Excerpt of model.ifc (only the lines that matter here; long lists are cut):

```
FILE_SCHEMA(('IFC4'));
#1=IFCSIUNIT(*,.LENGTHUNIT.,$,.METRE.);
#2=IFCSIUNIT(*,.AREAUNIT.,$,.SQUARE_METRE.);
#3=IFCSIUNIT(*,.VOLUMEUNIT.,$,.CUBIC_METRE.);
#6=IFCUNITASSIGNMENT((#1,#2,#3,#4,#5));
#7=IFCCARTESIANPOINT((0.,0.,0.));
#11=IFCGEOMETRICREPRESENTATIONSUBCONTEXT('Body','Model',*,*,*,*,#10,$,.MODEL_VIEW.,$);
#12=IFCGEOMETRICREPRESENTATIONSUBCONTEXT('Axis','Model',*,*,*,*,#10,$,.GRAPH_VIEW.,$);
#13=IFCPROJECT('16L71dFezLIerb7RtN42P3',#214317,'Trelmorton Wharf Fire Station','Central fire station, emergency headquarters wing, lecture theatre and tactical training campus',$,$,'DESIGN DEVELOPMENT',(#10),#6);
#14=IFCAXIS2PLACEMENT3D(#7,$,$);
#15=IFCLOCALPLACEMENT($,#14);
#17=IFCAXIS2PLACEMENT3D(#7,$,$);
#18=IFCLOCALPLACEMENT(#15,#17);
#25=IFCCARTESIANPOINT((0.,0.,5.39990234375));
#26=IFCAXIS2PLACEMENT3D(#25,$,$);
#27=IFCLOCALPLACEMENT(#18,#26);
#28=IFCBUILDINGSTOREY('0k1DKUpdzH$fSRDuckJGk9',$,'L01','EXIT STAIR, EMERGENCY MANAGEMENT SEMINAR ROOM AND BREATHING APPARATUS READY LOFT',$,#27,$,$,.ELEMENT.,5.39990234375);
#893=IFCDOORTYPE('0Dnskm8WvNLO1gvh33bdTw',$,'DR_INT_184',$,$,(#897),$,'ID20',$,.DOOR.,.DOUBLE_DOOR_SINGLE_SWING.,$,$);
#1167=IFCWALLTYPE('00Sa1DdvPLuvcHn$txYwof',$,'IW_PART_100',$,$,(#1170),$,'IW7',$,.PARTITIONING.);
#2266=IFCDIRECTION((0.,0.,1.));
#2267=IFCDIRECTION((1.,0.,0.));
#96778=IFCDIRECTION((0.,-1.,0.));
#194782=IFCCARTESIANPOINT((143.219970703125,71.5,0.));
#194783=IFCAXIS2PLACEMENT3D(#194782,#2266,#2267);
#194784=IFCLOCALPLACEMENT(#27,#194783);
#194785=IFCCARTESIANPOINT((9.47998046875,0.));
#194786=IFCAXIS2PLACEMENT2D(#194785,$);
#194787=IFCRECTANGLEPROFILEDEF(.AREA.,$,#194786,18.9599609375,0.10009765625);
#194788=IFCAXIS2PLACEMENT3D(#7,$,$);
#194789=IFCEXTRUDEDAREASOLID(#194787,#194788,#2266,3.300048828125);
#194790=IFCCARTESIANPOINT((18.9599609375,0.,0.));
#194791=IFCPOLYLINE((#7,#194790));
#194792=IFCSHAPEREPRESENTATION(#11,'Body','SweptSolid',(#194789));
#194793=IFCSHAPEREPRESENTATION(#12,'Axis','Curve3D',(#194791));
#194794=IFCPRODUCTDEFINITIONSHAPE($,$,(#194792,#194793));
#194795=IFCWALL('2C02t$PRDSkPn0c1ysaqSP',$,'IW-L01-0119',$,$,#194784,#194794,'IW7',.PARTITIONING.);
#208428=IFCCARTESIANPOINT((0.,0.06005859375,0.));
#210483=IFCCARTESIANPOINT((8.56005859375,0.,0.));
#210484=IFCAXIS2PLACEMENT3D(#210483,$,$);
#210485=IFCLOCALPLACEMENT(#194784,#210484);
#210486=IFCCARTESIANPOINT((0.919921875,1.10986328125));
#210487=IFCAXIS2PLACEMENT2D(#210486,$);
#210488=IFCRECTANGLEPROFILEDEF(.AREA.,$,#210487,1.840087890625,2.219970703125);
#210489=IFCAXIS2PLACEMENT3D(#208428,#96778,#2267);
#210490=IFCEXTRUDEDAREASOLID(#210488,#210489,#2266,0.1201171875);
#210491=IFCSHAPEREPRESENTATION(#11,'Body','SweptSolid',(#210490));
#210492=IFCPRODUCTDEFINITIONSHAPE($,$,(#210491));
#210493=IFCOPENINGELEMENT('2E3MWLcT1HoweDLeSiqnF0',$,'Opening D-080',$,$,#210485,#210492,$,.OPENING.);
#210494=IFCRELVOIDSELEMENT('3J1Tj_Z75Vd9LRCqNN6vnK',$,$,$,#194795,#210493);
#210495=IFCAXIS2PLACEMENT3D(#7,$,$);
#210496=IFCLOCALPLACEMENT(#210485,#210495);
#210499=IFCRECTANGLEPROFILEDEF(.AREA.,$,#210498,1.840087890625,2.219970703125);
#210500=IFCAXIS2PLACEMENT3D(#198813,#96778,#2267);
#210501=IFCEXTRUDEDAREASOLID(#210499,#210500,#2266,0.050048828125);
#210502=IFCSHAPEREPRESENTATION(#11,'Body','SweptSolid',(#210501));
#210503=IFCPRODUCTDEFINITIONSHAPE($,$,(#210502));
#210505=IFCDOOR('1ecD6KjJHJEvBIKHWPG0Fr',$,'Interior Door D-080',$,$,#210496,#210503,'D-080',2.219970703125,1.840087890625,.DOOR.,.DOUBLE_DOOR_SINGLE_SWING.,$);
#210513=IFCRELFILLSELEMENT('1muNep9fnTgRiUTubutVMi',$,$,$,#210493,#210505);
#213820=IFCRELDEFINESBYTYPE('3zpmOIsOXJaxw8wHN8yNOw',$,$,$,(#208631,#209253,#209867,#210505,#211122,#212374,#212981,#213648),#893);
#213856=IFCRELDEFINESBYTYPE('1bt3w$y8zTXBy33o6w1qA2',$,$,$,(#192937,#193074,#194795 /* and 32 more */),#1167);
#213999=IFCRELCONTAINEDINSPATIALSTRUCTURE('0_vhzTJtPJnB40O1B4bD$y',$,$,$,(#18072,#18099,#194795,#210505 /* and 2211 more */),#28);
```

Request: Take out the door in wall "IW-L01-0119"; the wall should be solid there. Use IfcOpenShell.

```python
import ifcopenshell
import ifcopenshell.api.feature
import ifcopenshell.api.root
import ifcopenshell.geom
import ifcopenshell.util.shape

model = ifcopenshell.open("model.ifc")
settings = ifcopenshell.geom.settings()


def volume(element):
    """Net volume in cubic metres, openings subtracted."""
    shape = ifcopenshell.geom.create_shape(settings, element)
    return ifcopenshell.util.shape.get_volume(shape.geometry)


door = model.by_id(210505)
opening = door.FillsVoids[0].RelatingOpeningElement
wall = opening.VoidsElements[0].RelatingBuildingElement
before = volume(wall)

ifcopenshell.api.root.remove_product(model, product=door)
ifcopenshell.api.feature.remove_feature(model, feature=opening)

after = volume(wall)

print(f"wall volume {before:.3f} -> {after:.3f} m3")

model.write("model_v2.ifc")
```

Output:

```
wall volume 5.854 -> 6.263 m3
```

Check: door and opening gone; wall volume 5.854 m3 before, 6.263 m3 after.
